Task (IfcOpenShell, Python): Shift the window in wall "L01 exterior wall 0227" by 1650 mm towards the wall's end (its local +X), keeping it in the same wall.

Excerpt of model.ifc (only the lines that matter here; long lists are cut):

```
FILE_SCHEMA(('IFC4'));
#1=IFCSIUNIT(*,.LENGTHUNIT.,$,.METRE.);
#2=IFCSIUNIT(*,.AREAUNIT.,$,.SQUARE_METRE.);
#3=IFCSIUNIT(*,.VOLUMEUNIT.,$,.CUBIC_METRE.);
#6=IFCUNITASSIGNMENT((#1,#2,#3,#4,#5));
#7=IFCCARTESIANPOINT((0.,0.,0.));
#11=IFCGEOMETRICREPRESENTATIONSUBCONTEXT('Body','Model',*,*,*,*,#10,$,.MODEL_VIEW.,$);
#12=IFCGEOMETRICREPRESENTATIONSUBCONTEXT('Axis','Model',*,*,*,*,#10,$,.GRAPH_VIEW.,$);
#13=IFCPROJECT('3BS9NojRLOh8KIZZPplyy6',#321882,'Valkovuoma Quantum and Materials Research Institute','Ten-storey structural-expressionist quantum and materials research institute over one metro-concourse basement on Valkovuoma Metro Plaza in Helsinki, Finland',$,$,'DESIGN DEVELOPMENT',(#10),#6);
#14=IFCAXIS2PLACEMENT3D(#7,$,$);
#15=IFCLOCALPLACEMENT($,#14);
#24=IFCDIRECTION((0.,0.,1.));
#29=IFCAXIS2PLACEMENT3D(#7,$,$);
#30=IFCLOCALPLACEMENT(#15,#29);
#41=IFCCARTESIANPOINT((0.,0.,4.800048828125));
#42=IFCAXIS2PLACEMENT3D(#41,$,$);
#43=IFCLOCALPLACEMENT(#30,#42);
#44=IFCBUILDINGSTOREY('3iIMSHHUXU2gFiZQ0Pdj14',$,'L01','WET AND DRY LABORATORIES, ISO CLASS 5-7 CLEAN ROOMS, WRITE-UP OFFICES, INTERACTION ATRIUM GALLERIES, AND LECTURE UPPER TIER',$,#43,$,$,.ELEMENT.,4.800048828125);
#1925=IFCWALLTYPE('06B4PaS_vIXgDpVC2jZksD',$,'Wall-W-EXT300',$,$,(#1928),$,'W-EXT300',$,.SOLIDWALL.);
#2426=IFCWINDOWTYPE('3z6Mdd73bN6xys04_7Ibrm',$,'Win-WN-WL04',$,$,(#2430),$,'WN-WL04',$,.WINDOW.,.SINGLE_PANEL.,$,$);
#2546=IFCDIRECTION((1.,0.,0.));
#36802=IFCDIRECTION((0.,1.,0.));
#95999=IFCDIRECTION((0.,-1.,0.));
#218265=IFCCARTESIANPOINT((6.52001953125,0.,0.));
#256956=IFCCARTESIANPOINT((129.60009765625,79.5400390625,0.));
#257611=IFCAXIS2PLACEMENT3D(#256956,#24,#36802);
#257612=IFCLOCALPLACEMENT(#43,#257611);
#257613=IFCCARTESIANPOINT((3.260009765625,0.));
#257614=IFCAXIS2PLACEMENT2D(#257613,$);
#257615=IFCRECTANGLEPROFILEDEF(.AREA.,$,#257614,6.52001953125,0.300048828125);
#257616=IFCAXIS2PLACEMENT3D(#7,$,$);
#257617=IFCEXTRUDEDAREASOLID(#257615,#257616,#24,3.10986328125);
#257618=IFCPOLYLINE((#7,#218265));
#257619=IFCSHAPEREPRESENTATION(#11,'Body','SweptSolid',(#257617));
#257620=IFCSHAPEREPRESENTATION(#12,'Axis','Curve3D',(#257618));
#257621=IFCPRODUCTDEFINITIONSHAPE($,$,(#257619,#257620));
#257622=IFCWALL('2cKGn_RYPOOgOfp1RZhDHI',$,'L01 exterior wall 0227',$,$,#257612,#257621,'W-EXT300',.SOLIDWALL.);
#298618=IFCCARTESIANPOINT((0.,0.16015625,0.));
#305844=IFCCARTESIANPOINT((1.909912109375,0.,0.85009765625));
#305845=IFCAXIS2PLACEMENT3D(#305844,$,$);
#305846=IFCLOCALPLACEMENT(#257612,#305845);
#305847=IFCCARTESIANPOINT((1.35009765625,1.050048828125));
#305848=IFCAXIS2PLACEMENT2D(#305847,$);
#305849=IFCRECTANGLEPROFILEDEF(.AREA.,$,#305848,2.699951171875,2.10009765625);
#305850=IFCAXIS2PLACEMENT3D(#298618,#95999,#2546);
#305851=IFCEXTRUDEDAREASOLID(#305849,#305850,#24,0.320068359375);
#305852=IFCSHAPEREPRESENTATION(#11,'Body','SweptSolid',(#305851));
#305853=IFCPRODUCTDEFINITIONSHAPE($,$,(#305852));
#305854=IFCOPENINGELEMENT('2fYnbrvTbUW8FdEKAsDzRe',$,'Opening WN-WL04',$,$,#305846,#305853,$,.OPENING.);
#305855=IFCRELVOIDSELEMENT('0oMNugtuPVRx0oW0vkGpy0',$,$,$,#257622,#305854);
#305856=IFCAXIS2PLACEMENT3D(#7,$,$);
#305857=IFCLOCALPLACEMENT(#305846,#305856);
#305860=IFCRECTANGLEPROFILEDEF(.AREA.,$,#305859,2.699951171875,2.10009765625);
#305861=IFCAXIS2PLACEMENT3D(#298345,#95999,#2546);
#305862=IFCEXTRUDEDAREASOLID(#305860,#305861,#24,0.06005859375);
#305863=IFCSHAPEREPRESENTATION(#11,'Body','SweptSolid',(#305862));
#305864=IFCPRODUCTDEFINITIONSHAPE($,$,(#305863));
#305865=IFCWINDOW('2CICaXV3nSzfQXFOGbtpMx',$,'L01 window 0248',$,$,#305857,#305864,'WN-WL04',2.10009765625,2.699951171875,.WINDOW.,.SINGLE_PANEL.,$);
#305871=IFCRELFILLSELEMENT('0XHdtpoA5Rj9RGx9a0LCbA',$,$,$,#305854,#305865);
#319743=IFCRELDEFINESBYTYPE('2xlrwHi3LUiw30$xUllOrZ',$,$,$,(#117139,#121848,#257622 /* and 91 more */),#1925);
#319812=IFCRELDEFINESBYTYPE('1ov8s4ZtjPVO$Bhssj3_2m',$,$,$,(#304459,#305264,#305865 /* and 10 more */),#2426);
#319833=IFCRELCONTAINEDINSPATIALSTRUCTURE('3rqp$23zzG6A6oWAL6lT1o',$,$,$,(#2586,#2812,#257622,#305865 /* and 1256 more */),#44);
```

```python
import ifcopenshell
import ifcopenshell.api.geometry
import ifcopenshell.util.placement

model = ifcopenshell.open("model.ifc")

window = model.by_guid("2CICaXV3nSzfQXFOGbtpMx")
opening = window.FillsVoids[0].RelatingOpeningElement
wall = opening.VoidsElements[0].RelatingBuildingElement

wall_matrix = ifcopenshell.util.placement.get_local_placement(wall.ObjectPlacement)
shift = wall_matrix[:3, 0] * 1.65
before = ifcopenshell.util.placement.get_local_placement(window.ObjectPlacement)[:3, 3].copy()

# The window is placed relative to its opening, so it follows when the opening moves.
matrix = ifcopenshell.util.placement.get_local_placement(opening.ObjectPlacement)
matrix[:3, 3] += shift
ifcopenshell.api.geometry.edit_object_placement(
    model, product=opening, matrix=matrix, is_si=False, should_transform_children=True
)

after = ifcopenshell.util.placement.get_local_placement(window.ObjectPlacement)[:3, 3]
print("window moved by", (after - before).round(3) + 0.0)

model.write("model_v2.ifc")
```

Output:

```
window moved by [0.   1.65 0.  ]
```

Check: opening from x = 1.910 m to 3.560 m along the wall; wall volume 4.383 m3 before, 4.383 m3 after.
